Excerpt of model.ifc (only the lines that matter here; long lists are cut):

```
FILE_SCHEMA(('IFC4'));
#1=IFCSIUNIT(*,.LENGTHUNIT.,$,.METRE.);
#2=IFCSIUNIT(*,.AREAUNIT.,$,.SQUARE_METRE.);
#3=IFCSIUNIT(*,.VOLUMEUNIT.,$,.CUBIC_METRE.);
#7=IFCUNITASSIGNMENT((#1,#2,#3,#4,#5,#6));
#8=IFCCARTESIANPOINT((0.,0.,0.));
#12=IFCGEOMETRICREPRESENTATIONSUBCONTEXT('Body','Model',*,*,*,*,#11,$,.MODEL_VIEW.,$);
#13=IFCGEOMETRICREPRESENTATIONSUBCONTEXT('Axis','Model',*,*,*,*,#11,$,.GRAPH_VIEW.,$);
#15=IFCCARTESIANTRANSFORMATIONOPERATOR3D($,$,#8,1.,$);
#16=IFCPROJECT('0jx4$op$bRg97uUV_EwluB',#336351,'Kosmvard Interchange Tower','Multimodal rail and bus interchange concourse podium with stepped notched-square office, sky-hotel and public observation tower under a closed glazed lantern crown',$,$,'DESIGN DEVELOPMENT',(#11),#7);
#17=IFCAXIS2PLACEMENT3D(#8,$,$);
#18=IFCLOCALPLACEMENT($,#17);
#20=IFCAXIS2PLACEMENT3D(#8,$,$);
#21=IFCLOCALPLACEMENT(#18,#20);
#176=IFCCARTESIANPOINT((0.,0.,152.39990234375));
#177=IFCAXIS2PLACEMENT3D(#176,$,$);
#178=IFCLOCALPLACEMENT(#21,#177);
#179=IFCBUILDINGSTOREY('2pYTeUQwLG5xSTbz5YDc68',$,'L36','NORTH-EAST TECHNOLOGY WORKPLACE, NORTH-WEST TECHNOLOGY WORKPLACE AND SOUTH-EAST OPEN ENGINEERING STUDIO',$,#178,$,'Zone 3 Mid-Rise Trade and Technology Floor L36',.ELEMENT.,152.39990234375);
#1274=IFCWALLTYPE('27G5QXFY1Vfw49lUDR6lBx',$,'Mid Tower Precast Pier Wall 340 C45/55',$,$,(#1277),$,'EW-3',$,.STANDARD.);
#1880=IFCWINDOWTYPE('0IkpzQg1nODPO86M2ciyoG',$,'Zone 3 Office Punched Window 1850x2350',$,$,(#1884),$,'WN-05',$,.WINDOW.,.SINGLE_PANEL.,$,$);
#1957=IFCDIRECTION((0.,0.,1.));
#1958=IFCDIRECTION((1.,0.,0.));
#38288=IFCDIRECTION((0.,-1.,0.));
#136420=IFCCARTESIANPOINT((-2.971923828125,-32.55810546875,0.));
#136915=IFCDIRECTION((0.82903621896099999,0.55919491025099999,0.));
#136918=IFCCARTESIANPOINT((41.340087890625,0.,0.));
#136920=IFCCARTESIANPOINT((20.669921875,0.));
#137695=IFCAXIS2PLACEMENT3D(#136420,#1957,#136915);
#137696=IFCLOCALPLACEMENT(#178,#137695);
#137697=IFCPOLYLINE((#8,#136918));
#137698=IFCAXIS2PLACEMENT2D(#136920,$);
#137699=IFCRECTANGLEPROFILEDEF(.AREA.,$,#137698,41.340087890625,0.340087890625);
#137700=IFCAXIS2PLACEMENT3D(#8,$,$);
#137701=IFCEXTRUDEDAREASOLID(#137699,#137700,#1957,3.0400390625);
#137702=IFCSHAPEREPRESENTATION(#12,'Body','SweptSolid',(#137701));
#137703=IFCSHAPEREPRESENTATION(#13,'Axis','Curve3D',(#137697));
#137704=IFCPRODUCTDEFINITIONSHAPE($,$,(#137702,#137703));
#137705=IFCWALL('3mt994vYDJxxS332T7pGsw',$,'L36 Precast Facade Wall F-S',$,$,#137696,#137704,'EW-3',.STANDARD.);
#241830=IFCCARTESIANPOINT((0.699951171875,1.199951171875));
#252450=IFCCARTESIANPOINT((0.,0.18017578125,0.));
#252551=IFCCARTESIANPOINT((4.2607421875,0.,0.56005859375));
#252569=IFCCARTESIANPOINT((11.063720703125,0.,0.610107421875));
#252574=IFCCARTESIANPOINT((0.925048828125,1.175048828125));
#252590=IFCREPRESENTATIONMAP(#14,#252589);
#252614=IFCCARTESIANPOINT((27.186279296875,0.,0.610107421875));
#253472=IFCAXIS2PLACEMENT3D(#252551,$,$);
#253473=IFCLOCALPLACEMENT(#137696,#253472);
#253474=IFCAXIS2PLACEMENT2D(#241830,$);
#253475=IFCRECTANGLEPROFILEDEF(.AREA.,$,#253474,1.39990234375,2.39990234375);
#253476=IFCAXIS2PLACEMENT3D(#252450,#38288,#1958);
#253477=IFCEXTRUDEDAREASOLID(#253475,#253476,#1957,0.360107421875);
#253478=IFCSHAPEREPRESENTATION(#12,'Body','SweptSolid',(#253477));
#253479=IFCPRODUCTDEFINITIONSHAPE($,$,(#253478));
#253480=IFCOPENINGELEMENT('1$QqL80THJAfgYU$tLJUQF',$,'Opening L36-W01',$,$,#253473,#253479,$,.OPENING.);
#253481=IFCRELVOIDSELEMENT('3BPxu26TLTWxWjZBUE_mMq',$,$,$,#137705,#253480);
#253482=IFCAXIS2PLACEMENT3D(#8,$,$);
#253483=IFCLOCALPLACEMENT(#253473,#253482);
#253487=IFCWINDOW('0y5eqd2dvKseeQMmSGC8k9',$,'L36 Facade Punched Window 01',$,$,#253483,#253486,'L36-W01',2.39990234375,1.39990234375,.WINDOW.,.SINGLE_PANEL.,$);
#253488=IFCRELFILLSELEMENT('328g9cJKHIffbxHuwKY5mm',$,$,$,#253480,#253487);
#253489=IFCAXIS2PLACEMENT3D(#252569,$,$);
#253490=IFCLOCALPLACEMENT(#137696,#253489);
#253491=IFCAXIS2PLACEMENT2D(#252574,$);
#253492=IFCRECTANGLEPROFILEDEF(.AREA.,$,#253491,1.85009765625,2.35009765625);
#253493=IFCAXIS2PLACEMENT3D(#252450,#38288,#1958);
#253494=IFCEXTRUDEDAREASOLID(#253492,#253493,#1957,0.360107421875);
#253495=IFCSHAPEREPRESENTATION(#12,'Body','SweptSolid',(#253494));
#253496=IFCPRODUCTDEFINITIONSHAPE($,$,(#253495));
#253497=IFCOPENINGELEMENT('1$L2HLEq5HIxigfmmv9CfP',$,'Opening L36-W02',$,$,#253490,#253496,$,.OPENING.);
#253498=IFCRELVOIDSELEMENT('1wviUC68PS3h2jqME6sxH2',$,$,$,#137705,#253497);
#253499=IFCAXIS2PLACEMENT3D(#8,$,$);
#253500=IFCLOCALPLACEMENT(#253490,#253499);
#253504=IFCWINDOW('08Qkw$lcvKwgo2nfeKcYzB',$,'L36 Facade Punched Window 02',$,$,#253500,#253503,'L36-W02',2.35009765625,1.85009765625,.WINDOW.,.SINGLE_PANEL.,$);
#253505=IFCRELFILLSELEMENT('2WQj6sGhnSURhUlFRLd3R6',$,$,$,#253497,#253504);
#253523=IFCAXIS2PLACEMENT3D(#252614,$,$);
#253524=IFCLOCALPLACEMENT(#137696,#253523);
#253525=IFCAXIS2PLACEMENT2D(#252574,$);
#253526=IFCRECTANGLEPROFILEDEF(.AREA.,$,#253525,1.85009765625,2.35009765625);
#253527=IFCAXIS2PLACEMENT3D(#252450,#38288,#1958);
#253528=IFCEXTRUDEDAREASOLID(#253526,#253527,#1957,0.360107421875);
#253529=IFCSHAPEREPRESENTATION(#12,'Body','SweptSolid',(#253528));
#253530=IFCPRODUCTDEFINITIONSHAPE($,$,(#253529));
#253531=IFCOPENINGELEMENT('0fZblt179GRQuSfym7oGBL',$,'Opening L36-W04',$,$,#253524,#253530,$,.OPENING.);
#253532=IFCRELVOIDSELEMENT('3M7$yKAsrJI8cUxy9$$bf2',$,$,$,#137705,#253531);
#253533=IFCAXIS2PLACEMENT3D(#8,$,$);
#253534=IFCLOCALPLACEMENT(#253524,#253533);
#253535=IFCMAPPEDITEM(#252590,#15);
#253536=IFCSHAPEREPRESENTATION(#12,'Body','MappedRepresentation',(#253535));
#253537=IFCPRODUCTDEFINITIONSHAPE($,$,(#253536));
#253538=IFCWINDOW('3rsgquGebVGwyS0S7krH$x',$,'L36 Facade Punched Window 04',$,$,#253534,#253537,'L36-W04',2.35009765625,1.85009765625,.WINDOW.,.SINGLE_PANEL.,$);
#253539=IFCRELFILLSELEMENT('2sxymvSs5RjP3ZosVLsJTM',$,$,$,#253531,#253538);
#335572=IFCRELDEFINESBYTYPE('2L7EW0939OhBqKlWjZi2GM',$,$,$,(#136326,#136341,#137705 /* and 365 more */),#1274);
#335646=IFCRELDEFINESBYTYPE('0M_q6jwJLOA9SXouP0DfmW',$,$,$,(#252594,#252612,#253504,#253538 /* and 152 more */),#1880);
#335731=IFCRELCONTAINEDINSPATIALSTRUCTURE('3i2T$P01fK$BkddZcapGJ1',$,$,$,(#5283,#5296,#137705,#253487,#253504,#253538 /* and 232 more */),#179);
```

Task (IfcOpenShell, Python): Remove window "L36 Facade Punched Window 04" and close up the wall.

```python
import ifcopenshell
import ifcopenshell.api.feature
import ifcopenshell.api.root
import ifcopenshell.geom
import ifcopenshell.util.shape

model = ifcopenshell.open("model.ifc")
settings = ifcopenshell.geom.settings()


def volume(element):
    """Net volume in cubic metres, openings subtracted."""
    shape = ifcopenshell.geom.create_shape(settings, element)
    return ifcopenshell.util.shape.get_volume(shape.geometry)


window = model.by_guid("3rsgquGebVGwyS0S7krH$x")
opening = window.FillsVoids[0].RelatingOpeningElement
wall = opening.VoidsElements[0].RelatingBuildingElement
before = volume(wall)

ifcopenshell.api.root.remove_product(model, product=window)
ifcopenshell.api.feature.remove_feature(model, feature=opening)

after = volume(wall)

print(f"wall volume {before:.3f} -> {after:.3f} m3")

model.write("model-out.ifc")
```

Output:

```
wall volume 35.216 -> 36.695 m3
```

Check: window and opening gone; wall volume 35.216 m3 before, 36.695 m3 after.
